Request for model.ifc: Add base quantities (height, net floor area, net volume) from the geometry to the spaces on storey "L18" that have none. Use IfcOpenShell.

First a look at what the model holds.

```python
import ifcopenshell
import ifcopenshell.util.element
import ifcopenshell.util.unit

model = ifcopenshell.open("model.ifc")
print(model.schema)
for unit_type in ("LENGTHUNIT", "AREAUNIT", "VOLUMEUNIT"):
    print(unit_type, ifcopenshell.util.unit.calculate_unit_scale(model, unit_type))
storey = next(s for s in model.by_type("IfcBuildingStorey") if s.Name == "L18")
spaces = [e for e in ifcopenshell.util.element.get_decomposition(storey) if e.is_a("IfcSpace")]
for e in sorted(spaces, key=lambda e: e.id()):
    print(e.id(), e.is_a(), e.Name, list(ifcopenshell.util.element.get_psets(e, qtos_only=True)), sep=" | ")
```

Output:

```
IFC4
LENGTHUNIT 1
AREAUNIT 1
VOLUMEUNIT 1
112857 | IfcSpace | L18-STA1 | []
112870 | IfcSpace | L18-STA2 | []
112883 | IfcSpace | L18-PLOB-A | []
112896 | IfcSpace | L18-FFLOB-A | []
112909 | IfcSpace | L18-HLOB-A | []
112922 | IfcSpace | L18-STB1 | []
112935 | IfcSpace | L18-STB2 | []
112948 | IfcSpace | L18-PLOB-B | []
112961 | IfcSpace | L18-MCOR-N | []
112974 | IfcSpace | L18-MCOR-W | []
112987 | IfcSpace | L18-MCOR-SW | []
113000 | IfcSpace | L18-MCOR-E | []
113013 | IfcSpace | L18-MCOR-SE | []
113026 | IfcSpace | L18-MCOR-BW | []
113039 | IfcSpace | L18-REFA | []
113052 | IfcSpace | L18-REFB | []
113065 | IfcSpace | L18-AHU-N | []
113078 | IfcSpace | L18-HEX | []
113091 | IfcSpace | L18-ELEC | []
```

```python
import ifcopenshell
import ifcopenshell.api.pset
import ifcopenshell.geom
import ifcopenshell.util.element
import ifcopenshell.util.shape
import ifcopenshell.util.unit

model = ifcopenshell.open("model.ifc")
unit_scale = ifcopenshell.util.unit.calculate_unit_scale(model)
area_scale = ifcopenshell.util.unit.calculate_unit_scale(model, "AREAUNIT")
volume_scale = ifcopenshell.util.unit.calculate_unit_scale(model, "VOLUMEUNIT")
settings = ifcopenshell.geom.settings()

storey = next(s for s in model.by_type("IfcBuildingStorey") if s.Name == "L18")
spaces = [e for e in ifcopenshell.util.element.get_decomposition(storey) if e.is_a("IfcSpace")]

for e in sorted(spaces, key=lambda e: e.id()):
    if ifcopenshell.util.element.get_psets(e, qtos_only=True, should_inherit=False):
        continue
    # Geometry comes back in metres, in the element's own axes.
    shape = ifcopenshell.geom.create_shape(settings, e)
    values = {
        "Height": ifcopenshell.util.shape.get_z(shape.geometry) / unit_scale,
        "NetFloorArea": ifcopenshell.util.shape.get_footprint_area(shape.geometry) / area_scale,
        "NetVolume": ifcopenshell.util.shape.get_volume(shape.geometry) / volume_scale,
    }
    qto = ifcopenshell.api.pset.add_qto(model, product=e, name="Qto_SpaceBaseQuantities")
    ifcopenshell.api.pset.edit_qto(model, qto=qto, properties=values)
    print(e.id(), {k: round(v, 3) for k, v in values.items()})

model.write("model_rev.ifc")
```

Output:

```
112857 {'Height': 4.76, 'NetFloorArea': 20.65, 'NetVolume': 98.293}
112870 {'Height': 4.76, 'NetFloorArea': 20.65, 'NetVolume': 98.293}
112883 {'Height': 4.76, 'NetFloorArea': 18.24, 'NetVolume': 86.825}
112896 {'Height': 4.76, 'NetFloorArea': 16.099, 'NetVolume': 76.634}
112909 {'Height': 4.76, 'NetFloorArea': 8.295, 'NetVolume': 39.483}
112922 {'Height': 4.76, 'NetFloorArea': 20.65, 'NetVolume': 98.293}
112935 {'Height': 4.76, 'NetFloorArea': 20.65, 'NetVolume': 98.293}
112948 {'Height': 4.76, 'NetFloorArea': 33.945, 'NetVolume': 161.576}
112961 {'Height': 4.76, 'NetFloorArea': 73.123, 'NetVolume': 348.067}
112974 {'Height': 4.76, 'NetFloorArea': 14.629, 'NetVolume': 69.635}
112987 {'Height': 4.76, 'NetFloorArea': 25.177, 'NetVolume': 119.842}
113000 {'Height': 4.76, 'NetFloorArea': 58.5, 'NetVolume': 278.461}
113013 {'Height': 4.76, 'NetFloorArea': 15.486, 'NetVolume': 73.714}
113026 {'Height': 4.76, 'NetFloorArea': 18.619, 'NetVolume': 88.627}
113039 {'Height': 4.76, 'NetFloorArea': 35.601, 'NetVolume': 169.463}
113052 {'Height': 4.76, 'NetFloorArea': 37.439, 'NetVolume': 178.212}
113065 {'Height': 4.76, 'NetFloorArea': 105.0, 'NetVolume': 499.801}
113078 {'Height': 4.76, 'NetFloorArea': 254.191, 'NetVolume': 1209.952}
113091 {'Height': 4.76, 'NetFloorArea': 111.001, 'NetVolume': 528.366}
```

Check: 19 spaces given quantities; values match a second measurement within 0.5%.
